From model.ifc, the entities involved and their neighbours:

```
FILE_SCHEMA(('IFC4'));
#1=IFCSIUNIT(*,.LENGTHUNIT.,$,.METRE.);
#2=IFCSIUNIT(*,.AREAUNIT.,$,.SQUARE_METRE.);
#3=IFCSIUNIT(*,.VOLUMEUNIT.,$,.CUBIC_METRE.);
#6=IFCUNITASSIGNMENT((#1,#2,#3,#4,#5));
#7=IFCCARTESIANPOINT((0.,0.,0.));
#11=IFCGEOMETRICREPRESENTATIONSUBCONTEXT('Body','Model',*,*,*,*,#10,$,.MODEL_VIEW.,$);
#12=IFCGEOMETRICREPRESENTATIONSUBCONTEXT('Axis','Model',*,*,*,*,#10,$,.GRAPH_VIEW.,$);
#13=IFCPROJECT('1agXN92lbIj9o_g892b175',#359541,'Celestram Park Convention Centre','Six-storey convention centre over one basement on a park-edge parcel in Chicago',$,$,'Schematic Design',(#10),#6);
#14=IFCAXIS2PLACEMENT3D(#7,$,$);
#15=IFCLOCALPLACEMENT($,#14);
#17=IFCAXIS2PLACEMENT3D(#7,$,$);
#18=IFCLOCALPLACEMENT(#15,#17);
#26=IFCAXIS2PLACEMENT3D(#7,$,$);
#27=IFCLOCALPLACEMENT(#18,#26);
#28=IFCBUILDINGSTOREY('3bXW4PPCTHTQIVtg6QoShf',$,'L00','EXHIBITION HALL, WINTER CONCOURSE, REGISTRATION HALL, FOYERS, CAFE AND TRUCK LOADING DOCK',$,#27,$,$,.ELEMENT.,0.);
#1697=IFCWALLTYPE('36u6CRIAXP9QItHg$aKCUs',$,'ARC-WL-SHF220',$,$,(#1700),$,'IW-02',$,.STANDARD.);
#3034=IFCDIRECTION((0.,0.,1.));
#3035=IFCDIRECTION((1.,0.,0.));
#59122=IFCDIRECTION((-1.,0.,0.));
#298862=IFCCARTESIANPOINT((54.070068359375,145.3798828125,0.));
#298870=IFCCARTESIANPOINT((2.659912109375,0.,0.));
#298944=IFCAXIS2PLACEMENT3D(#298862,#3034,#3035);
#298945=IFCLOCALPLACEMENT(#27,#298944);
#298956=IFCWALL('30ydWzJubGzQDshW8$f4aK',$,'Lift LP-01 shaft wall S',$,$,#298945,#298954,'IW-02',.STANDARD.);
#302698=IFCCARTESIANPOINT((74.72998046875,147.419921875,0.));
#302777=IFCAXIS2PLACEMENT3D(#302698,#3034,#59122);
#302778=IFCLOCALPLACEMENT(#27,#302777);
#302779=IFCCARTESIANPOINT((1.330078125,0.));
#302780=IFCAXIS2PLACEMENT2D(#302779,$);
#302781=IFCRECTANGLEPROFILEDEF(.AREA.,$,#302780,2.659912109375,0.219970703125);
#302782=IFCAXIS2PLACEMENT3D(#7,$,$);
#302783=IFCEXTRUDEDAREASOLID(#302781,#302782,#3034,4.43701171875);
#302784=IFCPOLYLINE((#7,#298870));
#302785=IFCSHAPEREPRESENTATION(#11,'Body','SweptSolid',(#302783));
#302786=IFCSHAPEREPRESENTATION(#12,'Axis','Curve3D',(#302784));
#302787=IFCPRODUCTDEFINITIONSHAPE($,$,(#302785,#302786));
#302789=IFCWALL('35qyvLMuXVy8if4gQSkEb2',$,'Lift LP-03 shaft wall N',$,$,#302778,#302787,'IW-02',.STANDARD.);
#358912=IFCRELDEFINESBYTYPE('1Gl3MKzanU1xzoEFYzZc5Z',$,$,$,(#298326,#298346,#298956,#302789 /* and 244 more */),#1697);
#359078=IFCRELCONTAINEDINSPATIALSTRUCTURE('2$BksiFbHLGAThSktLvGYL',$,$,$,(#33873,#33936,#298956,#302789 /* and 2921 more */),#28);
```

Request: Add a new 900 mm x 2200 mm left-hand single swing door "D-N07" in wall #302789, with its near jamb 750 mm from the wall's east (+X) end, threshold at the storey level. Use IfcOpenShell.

```python
import numpy as np
import ifcopenshell
import ifcopenshell.api.feature
import ifcopenshell.api.geometry
import ifcopenshell.api.root
import ifcopenshell.api.spatial
import ifcopenshell.geom
import ifcopenshell.util.element
import ifcopenshell.util.placement
import ifcopenshell.util.representation
import ifcopenshell.util.shape
import ifcopenshell.util.unit

model = ifcopenshell.open("model.ifc")
unit_scale = ifcopenshell.util.unit.calculate_unit_scale(model)
settings = ifcopenshell.geom.settings()


def volume(element):
    """Net volume in cubic metres, openings subtracted."""
    shape = ifcopenshell.geom.create_shape(settings, element)
    return ifcopenshell.util.shape.get_volume(shape.geometry)


wall = model.by_guid("35qyvLMuXVy8if4gQSkEb2")
storey = ifcopenshell.util.element.get_container(wall, ifc_class="IfcBuildingStorey")
context = ifcopenshell.util.representation.get_context(model, "Model", "Body", "MODEL_VIEW")
before = volume(wall)

width, height, from_end, sill = 0.9, 2.2, 0.75, 0.0  # metres

# The wall runs along its own X axis, and the end named is its -X end.
wall_shape = ifcopenshell.geom.create_shape(settings, wall)
x, y, z = ifcopenshell.util.shape.get_vertices(wall_shape.geometry).T
start = x.min() + from_end
face, thickness = float(y.min()), float(y.max() - y.min())
wall_matrix = ifcopenshell.util.placement.get_local_placement(wall.ObjectPlacement)
level = ifcopenshell.util.placement.get_local_placement(storey.ObjectPlacement)[2, 3]


def in_wall(x, y):
    """Placement at x, y metres in the wall's axes, at sill height."""
    matrix = wall_matrix.copy()
    matrix[:, 3] = wall_matrix @ np.array([x / unit_scale, y / unit_scale, 0.0, 1.0])
    matrix[2, 3] = level + sill / unit_scale
    return matrix


# Opening: a box that overshoots both wall faces by 50 mm.
opening = ifcopenshell.api.root.create_entity(model, ifc_class="IfcOpeningElement", predefined_type="OPENING")
box = ifcopenshell.api.geometry.add_wall_representation(
    model, context=context, length=width, height=height, thickness=thickness + 0.1
)
ifcopenshell.api.geometry.assign_representation(model, product=opening, representation=box)
ifcopenshell.api.geometry.edit_object_placement(model, product=opening, matrix=in_wall(start, face - 0.05), is_si=False)
ifcopenshell.api.feature.add_feature(model, feature=opening, element=wall)

door = ifcopenshell.api.root.create_entity(model, ifc_class="IfcDoor", name="D-N07", predefined_type="DOOR")
door.OverallWidth, door.OverallHeight = width / unit_scale, height / unit_scale
door.OperationType = "SINGLE_SWING_LEFT"
body = ifcopenshell.api.geometry.add_door_representation(
    model,
    context=context,
    overall_width=door.OverallWidth,
    overall_height=door.OverallHeight,
    operation_type="SINGLE_SWING_LEFT",
    lining_properties={"LiningDepth": thickness / unit_scale, "ThresholdDepth": thickness / unit_scale},
)
ifcopenshell.api.geometry.assign_representation(model, product=door, representation=body)
ifcopenshell.api.spatial.assign_container(model, products=[door], relating_structure=storey)
ifcopenshell.api.feature.add_filling(model, opening=opening, element=door)

# The lining spans the wall, so the door starts at the wall face.
ifcopenshell.api.geometry.edit_object_placement(model, product=door, matrix=in_wall(start, face), is_si=False)

after = volume(wall)

print(f"wall volume {before:.3f} -> {after:.3f} m3")

model.write("model_v2.ifc")
```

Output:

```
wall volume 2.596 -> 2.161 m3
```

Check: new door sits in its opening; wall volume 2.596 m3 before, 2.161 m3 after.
